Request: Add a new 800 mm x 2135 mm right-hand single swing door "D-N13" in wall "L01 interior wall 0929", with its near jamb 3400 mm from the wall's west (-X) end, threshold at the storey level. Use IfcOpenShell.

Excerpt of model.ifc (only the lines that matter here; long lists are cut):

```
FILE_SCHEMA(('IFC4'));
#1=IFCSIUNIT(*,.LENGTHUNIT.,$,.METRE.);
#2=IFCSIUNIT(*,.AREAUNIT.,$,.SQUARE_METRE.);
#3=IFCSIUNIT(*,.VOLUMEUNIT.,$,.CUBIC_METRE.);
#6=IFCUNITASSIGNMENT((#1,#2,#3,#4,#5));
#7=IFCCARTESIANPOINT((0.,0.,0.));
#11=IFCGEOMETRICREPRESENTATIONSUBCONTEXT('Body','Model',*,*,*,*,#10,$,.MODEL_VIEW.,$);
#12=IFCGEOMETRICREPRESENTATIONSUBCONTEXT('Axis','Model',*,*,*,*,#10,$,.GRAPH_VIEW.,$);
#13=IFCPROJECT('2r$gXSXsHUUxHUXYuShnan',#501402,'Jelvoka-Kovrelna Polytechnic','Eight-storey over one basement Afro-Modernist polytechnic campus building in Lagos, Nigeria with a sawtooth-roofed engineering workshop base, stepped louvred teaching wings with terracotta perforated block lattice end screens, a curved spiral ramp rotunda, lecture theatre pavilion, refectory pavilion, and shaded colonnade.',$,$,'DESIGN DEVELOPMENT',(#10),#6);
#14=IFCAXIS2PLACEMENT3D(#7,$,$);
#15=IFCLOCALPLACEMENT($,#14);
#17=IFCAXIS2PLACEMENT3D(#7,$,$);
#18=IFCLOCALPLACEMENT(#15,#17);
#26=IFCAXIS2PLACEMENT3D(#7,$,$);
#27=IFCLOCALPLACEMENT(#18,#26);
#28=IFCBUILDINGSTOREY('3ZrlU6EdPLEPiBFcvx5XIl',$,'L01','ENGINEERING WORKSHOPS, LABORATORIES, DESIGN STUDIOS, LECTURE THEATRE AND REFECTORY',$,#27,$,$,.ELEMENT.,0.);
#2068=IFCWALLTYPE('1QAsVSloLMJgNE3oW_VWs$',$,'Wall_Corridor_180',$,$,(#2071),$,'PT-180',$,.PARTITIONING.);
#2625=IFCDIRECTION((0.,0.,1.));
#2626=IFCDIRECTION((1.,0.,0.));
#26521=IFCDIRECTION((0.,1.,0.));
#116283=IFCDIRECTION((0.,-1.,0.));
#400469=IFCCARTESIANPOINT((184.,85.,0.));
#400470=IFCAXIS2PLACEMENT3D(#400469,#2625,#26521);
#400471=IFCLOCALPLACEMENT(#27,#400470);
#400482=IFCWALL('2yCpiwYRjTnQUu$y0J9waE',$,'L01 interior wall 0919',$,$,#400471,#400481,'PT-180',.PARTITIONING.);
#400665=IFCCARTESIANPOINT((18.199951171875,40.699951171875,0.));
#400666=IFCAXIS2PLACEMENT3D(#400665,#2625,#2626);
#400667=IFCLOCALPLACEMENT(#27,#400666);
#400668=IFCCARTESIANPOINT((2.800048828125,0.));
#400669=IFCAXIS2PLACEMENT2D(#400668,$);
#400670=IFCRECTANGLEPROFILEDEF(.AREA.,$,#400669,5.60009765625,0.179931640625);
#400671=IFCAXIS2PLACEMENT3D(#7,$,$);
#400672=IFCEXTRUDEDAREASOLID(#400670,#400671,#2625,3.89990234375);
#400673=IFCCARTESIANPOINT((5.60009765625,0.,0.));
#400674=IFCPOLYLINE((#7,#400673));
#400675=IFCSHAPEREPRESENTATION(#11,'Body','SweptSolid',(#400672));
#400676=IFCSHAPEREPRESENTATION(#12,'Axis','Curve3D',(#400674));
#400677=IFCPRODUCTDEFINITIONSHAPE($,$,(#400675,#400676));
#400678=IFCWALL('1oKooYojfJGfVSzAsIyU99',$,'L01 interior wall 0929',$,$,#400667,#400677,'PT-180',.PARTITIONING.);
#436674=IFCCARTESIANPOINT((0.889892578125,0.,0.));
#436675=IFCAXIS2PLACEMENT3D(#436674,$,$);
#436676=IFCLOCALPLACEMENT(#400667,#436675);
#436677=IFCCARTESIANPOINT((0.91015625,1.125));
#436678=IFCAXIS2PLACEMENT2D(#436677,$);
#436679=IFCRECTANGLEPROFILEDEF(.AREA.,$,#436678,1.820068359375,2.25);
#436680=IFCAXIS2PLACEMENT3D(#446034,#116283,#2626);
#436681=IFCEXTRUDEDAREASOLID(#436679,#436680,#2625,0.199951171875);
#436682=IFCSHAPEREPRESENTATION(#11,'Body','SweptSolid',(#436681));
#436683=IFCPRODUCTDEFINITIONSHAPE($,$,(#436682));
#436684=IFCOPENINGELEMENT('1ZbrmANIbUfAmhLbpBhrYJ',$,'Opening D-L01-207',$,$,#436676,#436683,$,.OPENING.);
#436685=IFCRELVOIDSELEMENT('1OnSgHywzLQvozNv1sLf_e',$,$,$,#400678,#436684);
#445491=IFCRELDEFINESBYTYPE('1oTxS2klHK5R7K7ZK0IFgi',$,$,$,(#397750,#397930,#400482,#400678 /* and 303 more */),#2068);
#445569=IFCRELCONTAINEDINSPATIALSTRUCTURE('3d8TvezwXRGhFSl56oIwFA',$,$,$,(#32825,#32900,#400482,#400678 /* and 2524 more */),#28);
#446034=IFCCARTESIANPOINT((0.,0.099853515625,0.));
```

```python
import numpy as np
import ifcopenshell
import ifcopenshell.api.feature
import ifcopenshell.api.geometry
import ifcopenshell.api.root
import ifcopenshell.api.spatial
import ifcopenshell.geom
import ifcopenshell.util.element
import ifcopenshell.util.placement
import ifcopenshell.util.representation
import ifcopenshell.util.shape
import ifcopenshell.util.unit

model = ifcopenshell.open("model.ifc")
unit_scale = ifcopenshell.util.unit.calculate_unit_scale(model)
settings = ifcopenshell.geom.settings()


def volume(element):
    """Net volume in cubic metres, openings subtracted."""
    shape = ifcopenshell.geom.create_shape(settings, element)
    return ifcopenshell.util.shape.get_volume(shape.geometry)


wall = model.by_id(400678)
storey = ifcopenshell.util.element.get_container(wall, ifc_class="IfcBuildingStorey")
context = ifcopenshell.util.representation.get_context(model, "Model", "Body", "MODEL_VIEW")
before = volume(wall)

width, height, from_end, sill = 0.8, 2.135, 3.4, 0.0  # metres

# The wall runs along its own X axis, and the end named is its -X end.
wall_shape = ifcopenshell.geom.create_shape(settings, wall)
x, y, z = ifcopenshell.util.shape.get_vertices(wall_shape.geometry).T
start = x.min() + from_end
face, thickness = float(y.min()), float(y.max() - y.min())
wall_matrix = ifcopenshell.util.placement.get_local_placement(wall.ObjectPlacement)
level = ifcopenshell.util.placement.get_local_placement(storey.ObjectPlacement)[2, 3]


def in_wall(x, y):
    """Placement at x, y metres in the wall's axes, at sill height."""
    matrix = wall_matrix.copy()
    matrix[:, 3] = wall_matrix @ np.array([x / unit_scale, y / unit_scale, 0.0, 1.0])
    matrix[2, 3] = level + sill / unit_scale
    return matrix


# Opening: a box that overshoots both wall faces by 50 mm.
opening = ifcopenshell.api.root.create_entity(model, ifc_class="IfcOpeningElement", predefined_type="OPENING")
box = ifcopenshell.api.geometry.add_wall_representation(
    model, context=context, length=width, height=height, thickness=thickness + 0.1
)
ifcopenshell.api.geometry.assign_representation(model, product=opening, representation=box)
ifcopenshell.api.geometry.edit_object_placement(model, product=opening, matrix=in_wall(start, face - 0.05), is_si=False)
ifcopenshell.api.feature.add_feature(model, feature=opening, element=wall)

door = ifcopenshell.api.root.create_entity(model, ifc_class="IfcDoor", name="D-N13", predefined_type="DOOR")
door.OverallWidth, door.OverallHeight = width / unit_scale, height / unit_scale
door.OperationType = "SINGLE_SWING_RIGHT"
body = ifcopenshell.api.geometry.add_door_representation(
    model,
    context=context,
    overall_width=door.OverallWidth,
    overall_height=door.OverallHeight,
    operation_type="SINGLE_SWING_RIGHT",
    lining_properties={"LiningDepth": thickness / unit_scale, "ThresholdDepth": thickness / unit_scale},
)
ifcopenshell.api.geometry.assign_representation(model, product=door, representation=body)
ifcopenshell.api.spatial.assign_container(model, products=[door], relating_structure=storey)
ifcopenshell.api.feature.add_filling(model, opening=opening, element=door)

# The lining spans the wall, so the door starts at the wall face.
ifcopenshell.api.geometry.edit_object_placement(model, product=door, matrix=in_wall(start, face), is_si=False)

after = volume(wall)

print(f"wall volume {before:.3f} -> {after:.3f} m3")

model.write("model_v2.ifc")
```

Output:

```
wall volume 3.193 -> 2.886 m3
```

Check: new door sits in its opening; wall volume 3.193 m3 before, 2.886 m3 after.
